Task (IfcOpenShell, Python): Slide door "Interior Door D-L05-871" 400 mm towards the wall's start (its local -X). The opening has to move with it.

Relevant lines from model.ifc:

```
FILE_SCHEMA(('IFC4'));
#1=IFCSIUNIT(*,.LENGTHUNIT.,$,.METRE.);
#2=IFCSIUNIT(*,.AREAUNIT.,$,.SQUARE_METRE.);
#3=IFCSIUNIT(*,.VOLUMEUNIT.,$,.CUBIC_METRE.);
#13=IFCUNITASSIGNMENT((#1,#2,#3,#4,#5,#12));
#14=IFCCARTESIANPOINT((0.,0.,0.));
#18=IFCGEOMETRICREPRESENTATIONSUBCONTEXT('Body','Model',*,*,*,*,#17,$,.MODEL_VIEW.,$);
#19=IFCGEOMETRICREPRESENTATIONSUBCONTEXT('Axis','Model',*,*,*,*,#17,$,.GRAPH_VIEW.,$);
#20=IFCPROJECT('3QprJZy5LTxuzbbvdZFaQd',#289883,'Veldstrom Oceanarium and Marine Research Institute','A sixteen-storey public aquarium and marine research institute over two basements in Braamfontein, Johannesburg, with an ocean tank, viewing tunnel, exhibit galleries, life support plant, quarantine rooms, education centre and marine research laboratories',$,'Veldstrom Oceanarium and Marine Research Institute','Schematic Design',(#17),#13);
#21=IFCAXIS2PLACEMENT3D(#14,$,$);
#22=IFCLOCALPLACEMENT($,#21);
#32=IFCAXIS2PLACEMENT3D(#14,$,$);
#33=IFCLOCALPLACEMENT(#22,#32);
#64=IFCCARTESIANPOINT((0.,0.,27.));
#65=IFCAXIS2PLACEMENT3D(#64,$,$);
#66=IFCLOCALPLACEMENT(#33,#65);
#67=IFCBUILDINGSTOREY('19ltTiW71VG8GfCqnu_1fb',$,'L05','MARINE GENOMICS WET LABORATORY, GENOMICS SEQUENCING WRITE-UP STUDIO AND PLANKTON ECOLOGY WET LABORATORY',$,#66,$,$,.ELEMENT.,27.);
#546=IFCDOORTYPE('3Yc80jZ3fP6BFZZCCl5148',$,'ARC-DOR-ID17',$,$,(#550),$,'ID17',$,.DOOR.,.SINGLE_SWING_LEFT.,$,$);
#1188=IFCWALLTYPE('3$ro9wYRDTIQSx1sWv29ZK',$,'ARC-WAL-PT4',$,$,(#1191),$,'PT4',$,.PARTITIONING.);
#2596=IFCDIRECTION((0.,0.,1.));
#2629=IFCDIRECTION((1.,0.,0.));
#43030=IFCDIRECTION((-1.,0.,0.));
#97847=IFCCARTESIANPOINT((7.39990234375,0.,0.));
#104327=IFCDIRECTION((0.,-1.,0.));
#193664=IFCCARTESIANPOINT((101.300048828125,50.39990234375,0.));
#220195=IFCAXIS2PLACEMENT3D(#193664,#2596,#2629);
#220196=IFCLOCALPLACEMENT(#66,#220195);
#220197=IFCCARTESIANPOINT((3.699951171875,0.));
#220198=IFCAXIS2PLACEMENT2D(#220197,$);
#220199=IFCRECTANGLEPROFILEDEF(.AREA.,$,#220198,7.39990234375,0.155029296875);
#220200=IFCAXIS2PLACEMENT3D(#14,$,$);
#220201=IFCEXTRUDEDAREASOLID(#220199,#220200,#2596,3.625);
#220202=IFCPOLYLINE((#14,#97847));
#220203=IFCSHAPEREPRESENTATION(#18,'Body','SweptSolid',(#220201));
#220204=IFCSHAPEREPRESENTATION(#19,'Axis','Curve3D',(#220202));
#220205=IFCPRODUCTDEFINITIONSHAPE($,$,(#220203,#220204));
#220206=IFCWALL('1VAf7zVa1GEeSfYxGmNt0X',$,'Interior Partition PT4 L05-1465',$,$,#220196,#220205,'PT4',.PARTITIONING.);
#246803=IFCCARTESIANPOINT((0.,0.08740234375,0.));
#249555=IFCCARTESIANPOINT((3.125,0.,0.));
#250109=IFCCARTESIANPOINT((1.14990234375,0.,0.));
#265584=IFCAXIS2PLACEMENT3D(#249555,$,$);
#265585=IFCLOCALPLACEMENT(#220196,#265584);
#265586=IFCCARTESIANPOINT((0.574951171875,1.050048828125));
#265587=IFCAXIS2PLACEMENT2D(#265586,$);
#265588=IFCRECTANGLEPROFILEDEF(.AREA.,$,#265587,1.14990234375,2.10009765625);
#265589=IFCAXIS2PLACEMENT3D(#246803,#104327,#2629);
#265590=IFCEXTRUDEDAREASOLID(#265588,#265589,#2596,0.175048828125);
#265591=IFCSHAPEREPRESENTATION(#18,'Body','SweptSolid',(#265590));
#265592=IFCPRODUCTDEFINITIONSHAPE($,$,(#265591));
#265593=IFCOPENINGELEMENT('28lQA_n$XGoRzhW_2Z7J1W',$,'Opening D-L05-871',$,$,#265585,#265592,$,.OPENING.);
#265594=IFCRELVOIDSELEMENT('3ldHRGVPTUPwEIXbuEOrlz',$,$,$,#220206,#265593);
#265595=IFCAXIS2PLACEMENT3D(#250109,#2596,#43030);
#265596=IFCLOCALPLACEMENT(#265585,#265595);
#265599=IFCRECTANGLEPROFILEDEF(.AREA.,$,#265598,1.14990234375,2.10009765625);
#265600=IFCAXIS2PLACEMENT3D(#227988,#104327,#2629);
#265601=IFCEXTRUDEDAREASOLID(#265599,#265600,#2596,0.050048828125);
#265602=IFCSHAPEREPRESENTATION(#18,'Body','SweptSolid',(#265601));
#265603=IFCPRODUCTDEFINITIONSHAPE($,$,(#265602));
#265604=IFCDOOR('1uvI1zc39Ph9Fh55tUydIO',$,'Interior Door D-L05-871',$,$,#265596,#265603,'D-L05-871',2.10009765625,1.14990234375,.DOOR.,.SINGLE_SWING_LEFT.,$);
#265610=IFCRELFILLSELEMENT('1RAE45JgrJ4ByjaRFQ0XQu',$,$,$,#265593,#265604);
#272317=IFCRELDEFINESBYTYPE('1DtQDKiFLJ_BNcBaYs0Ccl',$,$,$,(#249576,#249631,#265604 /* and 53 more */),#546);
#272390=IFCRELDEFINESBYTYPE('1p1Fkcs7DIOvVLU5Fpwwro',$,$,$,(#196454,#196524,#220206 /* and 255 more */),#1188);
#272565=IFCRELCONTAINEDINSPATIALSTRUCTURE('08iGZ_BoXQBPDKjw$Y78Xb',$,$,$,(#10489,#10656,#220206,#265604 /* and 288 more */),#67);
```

```python
import ifcopenshell
import ifcopenshell.api.geometry
import ifcopenshell.util.placement
import ifcopenshell.util.unit

model = ifcopenshell.open("model.ifc")
unit_scale = ifcopenshell.util.unit.calculate_unit_scale(model)

door = model.by_id(265604)
opening = door.FillsVoids[0].RelatingOpeningElement
wall = opening.VoidsElements[0].RelatingBuildingElement

wall_matrix = ifcopenshell.util.placement.get_local_placement(wall.ObjectPlacement)
shift = wall_matrix[:3, 0] * -0.4 / unit_scale
before = ifcopenshell.util.placement.get_local_placement(door.ObjectPlacement)[:3, 3].copy()

# The door is placed relative to its opening, so it follows when the opening moves.
matrix = ifcopenshell.util.placement.get_local_placement(opening.ObjectPlacement)
matrix[:3, 3] += shift
ifcopenshell.api.geometry.edit_object_placement(
    model, product=opening, matrix=matrix, is_si=False, should_transform_children=True
)

after = ifcopenshell.util.placement.get_local_placement(door.ObjectPlacement)[:3, 3]
print("door moved by", (after - before).round(3) + 0.0)

model.write("model_v2.ifc")
```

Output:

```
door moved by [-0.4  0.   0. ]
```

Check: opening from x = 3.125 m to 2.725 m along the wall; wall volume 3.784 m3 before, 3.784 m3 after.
